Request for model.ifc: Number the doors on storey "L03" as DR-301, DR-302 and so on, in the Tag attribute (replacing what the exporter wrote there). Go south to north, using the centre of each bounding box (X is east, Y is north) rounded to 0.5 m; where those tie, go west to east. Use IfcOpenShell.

First a look at what the model holds.

```python
import ifcopenshell
import ifcopenshell.util.element
import ifcopenshell.util.placement

model = ifcopenshell.open("model.ifc")
print(model.schema)
storey = next(s for s in model.by_type("IfcBuildingStorey") if s.Name == "L03")
doors = [e for e in ifcopenshell.util.element.get_decomposition(storey) if e.is_a("IfcDoor")]
for e in sorted(doors, key=lambda e: e.id()):
    origin = ifcopenshell.util.placement.get_local_placement(e.ObjectPlacement)[:3, 3]
    print(e.id(), e.Tag, e.Name, origin.round(2) + 0.0, sep=" | ")
```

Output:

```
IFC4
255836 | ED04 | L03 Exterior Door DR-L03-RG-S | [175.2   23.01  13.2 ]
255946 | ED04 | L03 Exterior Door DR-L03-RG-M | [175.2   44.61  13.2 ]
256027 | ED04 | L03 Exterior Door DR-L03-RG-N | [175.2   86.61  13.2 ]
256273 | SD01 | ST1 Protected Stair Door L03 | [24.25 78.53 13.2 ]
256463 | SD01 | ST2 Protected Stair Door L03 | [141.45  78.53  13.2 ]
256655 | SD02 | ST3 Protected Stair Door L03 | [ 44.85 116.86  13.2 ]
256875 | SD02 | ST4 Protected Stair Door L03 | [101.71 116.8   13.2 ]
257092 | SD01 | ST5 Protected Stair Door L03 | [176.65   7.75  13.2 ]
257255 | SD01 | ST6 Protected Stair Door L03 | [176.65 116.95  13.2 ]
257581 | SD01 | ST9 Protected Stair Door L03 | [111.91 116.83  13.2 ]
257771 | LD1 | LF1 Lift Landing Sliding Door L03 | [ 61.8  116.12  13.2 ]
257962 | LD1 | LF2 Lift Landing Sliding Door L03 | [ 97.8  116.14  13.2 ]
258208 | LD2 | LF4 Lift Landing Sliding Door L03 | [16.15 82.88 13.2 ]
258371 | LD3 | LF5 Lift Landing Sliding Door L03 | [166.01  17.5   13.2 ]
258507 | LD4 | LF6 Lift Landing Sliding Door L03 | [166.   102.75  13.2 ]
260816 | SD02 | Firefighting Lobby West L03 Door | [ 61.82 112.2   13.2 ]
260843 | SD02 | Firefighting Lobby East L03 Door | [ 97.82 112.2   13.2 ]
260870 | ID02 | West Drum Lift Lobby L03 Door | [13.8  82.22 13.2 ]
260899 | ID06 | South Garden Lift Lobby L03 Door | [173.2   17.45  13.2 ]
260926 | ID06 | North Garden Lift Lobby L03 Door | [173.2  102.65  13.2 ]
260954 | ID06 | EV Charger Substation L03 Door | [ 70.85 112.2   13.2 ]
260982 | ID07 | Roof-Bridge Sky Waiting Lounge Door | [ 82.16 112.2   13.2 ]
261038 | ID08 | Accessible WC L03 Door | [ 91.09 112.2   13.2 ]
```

```python
import ifcopenshell
import ifcopenshell.geom
import ifcopenshell.util.element
import ifcopenshell.util.shape

model = ifcopenshell.open("model.ifc")
settings = ifcopenshell.geom.settings()
settings.set("use-world-coords", True)


def centre(element):
    shape = ifcopenshell.geom.create_shape(settings, element)
    return ifcopenshell.util.shape.get_bbox_centroid(shape.geometry)


storey = next(s for s in model.by_type("IfcBuildingStorey") if s.Name == "L03")
doors = [e for e in ifcopenshell.util.element.get_decomposition(storey) if e.is_a("IfcDoor")]

# Insertion points can sit at a corner or the storey origin, so sort by the geometry (in metres).
centres = {e: centre(e) for e in doors}
doors.sort(key=lambda e: (round(centres[e][1] / 0.5), centres[e][0]))

for i, e in enumerate(doors, start=1):
    number = f"DR-3{i:02d}"
    e.Tag = number
    print(e.id(), number)

model.write("model_updated.ifc")
```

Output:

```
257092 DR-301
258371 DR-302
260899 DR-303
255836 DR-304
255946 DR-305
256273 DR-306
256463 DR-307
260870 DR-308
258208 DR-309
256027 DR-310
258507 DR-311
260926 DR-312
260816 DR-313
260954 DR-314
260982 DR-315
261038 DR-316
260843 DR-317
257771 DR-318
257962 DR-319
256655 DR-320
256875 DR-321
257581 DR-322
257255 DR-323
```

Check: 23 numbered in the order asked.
